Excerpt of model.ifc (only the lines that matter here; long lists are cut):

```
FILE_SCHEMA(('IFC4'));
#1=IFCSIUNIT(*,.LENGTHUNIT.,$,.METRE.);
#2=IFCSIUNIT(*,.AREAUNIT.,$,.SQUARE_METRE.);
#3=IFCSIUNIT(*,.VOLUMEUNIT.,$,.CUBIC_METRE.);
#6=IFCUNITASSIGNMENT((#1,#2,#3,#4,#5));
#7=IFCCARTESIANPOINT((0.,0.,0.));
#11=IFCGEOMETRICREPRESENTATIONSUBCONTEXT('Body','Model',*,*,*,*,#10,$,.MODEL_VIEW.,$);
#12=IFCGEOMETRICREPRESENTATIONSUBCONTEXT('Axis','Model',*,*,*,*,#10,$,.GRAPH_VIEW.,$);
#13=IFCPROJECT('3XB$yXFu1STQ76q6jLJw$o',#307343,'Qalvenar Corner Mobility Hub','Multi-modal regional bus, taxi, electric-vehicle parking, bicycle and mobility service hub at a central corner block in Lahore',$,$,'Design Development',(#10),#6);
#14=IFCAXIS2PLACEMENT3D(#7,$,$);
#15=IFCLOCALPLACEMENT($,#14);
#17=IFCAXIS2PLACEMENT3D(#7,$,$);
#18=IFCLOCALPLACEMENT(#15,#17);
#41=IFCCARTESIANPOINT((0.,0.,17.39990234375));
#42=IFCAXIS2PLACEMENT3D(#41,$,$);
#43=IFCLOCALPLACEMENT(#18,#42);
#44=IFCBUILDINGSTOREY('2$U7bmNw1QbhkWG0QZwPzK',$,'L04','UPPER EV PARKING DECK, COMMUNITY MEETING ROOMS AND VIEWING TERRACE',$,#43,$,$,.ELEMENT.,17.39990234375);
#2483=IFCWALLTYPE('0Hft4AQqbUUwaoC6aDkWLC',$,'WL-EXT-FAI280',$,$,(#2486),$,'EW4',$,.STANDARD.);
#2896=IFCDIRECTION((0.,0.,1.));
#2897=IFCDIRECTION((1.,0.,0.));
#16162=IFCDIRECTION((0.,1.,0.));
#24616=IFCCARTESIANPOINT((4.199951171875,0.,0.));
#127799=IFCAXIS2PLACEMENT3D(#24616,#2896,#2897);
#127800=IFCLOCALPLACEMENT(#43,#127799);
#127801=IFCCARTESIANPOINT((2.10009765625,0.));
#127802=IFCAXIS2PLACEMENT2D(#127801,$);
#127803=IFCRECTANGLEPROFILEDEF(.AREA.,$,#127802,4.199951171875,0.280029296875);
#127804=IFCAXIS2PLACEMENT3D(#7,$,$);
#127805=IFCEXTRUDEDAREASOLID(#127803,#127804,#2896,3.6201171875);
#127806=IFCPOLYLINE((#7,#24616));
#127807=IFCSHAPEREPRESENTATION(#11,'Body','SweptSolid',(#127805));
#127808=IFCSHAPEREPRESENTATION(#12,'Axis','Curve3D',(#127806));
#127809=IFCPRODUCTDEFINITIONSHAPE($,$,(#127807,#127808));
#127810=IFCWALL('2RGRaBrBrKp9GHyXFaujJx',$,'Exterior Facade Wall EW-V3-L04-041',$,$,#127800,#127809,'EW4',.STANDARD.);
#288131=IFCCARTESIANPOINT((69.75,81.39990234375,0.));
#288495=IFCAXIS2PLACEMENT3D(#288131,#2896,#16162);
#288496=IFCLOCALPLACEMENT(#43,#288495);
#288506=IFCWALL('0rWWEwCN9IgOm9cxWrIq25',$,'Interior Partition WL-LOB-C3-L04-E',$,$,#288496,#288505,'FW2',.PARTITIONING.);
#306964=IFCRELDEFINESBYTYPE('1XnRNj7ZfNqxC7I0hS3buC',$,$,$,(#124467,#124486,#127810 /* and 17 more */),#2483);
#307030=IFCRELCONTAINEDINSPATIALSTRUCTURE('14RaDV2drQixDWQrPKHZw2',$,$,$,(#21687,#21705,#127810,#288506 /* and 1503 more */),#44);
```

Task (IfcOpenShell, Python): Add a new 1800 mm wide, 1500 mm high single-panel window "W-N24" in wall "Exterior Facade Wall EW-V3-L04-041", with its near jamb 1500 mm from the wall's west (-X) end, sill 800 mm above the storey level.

```python
import numpy as np
import ifcopenshell
import ifcopenshell.api.feature
import ifcopenshell.api.geometry
import ifcopenshell.api.root
import ifcopenshell.api.spatial
import ifcopenshell.geom
import ifcopenshell.util.element
import ifcopenshell.util.placement
import ifcopenshell.util.representation
import ifcopenshell.util.shape
import ifcopenshell.util.unit

model = ifcopenshell.open("model.ifc")
unit_scale = ifcopenshell.util.unit.calculate_unit_scale(model)
settings = ifcopenshell.geom.settings()


def volume(element):
    """Net volume in cubic metres, openings subtracted."""
    shape = ifcopenshell.geom.create_shape(settings, element)
    return ifcopenshell.util.shape.get_volume(shape.geometry)


wall = model.by_guid("2RGRaBrBrKp9GHyXFaujJx")
storey = ifcopenshell.util.element.get_container(wall, ifc_class="IfcBuildingStorey")
context = ifcopenshell.util.representation.get_context(model, "Model", "Body", "MODEL_VIEW")
before = volume(wall)

width, height, from_end, sill = 1.8, 1.5, 1.5, 0.8  # metres

# The wall runs along its own X axis, and the end named is its -X end.
wall_shape = ifcopenshell.geom.create_shape(settings, wall)
x, y, z = ifcopenshell.util.shape.get_vertices(wall_shape.geometry).T
start = x.min() + from_end
face, thickness = float(y.min()), float(y.max() - y.min())
wall_matrix = ifcopenshell.util.placement.get_local_placement(wall.ObjectPlacement)
level = ifcopenshell.util.placement.get_local_placement(storey.ObjectPlacement)[2, 3]


def in_wall(x, y):
    """Placement at x, y metres in the wall's axes, at sill height."""
    matrix = wall_matrix.copy()
    matrix[:, 3] = wall_matrix @ np.array([x / unit_scale, y / unit_scale, 0.0, 1.0])
    matrix[2, 3] = level + sill / unit_scale
    return matrix


# Opening: a box that overshoots both wall faces by 50 mm.
opening = ifcopenshell.api.root.create_entity(model, ifc_class="IfcOpeningElement", predefined_type="OPENING")
box = ifcopenshell.api.geometry.add_wall_representation(
    model, context=context, length=width, height=height, thickness=thickness + 0.1
)
ifcopenshell.api.geometry.assign_representation(model, product=opening, representation=box)
ifcopenshell.api.geometry.edit_object_placement(model, product=opening, matrix=in_wall(start, face - 0.05), is_si=False)
ifcopenshell.api.feature.add_feature(model, feature=opening, element=wall)

window = ifcopenshell.api.root.create_entity(model, ifc_class="IfcWindow", name="W-N24", predefined_type="WINDOW")
window.OverallWidth, window.OverallHeight = width / unit_scale, height / unit_scale
window.PartitioningType = "SINGLE_PANEL"
body = ifcopenshell.api.geometry.add_window_representation(
    model,
    context=context,
    overall_width=window.OverallWidth,
    overall_height=window.OverallHeight,
    partition_type="SINGLE_PANEL",
)
ifcopenshell.api.geometry.assign_representation(model, product=window, representation=body)
ifcopenshell.api.spatial.assign_container(model, products=[window], relating_structure=storey)
ifcopenshell.api.feature.add_filling(model, opening=opening, element=window)

# Centre the window in the wall's thickness.
ifcopenshell.api.geometry.edit_object_placement(model, product=window, matrix=in_wall(start, face), is_si=False)
window_shape = ifcopenshell.geom.create_shape(settings, window)
depth = ifcopenshell.util.shape.get_vertices(window_shape.geometry)[:, 1]
offset = face + thickness / 2 - (depth.min() + depth.max()) / 2
ifcopenshell.api.geometry.edit_object_placement(model, product=window, matrix=in_wall(start, offset), is_si=False)

after = volume(wall)

print(f"wall volume {before:.3f} -> {after:.3f} m3")

model.write("model_edited.ifc")
```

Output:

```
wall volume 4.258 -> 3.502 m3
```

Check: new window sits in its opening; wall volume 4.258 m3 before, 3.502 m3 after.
